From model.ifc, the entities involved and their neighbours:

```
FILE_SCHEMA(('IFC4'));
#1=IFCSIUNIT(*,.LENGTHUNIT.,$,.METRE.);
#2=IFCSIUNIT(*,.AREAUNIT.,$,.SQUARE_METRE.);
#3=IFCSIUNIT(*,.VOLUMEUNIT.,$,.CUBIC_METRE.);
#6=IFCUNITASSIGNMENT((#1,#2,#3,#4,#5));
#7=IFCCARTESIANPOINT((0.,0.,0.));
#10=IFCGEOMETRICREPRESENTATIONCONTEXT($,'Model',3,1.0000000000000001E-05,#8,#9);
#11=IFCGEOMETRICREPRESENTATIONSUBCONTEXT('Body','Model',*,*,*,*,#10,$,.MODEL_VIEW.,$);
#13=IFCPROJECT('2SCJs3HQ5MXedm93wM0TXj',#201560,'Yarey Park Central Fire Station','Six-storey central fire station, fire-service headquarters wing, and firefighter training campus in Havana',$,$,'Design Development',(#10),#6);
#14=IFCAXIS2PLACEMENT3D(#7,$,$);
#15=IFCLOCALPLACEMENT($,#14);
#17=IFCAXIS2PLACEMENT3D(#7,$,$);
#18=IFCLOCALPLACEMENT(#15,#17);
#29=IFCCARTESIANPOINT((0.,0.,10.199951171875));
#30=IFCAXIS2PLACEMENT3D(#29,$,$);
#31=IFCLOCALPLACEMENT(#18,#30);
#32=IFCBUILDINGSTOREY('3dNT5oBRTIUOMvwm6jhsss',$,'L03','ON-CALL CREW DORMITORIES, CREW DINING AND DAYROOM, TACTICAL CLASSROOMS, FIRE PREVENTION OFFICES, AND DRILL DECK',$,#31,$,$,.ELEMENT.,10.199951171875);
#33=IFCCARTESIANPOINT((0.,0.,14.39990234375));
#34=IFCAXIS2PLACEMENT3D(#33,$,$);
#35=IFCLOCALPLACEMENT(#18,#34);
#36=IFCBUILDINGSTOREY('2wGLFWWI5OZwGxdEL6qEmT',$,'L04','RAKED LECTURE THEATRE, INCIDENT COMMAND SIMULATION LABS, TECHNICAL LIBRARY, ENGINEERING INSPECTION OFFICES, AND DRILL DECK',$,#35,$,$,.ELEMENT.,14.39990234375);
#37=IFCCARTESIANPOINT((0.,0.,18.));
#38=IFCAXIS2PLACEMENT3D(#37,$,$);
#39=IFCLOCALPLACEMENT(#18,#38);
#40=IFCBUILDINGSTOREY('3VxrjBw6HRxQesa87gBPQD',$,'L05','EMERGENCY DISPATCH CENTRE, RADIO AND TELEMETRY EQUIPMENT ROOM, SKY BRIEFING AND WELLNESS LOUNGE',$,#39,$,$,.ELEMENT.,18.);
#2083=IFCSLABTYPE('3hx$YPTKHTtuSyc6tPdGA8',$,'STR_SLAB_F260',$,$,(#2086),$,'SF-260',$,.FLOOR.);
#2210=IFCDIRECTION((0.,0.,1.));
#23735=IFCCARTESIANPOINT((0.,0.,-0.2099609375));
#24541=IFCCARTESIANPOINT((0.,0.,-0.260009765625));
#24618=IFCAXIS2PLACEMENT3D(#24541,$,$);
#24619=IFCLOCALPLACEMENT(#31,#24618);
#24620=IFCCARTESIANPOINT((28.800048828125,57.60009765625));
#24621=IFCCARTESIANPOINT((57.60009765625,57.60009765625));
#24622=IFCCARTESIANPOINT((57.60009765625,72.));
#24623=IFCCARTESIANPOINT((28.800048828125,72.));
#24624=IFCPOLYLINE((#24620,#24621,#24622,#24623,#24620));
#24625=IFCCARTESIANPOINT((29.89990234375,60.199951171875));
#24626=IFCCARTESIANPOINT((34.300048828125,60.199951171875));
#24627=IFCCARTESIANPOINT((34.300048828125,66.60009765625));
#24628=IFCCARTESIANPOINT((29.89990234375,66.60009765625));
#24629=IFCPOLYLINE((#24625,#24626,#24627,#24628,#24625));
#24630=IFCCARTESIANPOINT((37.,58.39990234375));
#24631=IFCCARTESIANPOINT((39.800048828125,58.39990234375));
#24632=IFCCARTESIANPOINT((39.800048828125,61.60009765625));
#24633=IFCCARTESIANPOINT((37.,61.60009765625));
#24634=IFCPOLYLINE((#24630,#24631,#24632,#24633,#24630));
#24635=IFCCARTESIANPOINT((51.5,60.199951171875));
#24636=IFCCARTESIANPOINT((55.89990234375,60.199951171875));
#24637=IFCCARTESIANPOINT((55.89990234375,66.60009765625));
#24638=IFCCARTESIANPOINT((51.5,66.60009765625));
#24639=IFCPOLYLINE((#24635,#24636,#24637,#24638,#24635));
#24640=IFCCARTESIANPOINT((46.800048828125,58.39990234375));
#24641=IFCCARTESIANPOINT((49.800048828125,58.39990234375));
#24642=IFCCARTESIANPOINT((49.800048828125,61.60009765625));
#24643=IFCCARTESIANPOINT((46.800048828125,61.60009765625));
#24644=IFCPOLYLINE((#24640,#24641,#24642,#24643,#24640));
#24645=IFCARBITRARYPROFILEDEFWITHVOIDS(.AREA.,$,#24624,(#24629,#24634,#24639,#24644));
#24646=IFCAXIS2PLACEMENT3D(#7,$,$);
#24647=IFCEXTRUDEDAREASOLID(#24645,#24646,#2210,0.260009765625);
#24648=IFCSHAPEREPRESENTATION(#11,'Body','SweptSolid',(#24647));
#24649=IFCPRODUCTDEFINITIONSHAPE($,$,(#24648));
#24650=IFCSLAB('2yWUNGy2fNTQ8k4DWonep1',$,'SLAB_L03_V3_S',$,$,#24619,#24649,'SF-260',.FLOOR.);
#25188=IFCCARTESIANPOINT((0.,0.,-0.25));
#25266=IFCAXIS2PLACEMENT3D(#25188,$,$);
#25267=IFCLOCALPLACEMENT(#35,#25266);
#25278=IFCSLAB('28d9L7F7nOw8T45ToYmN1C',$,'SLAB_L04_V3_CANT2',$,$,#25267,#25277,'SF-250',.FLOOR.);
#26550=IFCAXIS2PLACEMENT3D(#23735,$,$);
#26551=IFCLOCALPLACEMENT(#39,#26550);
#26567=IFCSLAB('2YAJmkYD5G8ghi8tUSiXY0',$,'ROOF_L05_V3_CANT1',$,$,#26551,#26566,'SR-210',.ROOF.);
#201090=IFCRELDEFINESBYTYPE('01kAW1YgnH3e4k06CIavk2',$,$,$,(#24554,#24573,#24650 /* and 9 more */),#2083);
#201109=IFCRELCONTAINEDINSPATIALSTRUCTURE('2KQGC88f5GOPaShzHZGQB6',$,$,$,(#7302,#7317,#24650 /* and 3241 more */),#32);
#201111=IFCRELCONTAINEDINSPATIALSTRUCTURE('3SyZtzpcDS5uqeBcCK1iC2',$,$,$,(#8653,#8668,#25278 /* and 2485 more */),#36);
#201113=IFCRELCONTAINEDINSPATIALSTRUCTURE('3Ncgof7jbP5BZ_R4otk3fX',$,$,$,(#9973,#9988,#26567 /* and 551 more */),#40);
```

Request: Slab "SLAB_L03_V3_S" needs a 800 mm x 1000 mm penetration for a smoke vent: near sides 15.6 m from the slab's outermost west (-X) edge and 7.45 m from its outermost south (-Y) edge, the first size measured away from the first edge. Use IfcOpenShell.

```python
import numpy as np
import ifcopenshell
import ifcopenshell.api.feature
import ifcopenshell.api.geometry
import ifcopenshell.api.root
import ifcopenshell.geom
import ifcopenshell.util.placement
import ifcopenshell.util.representation
import ifcopenshell.util.shape
import ifcopenshell.util.unit

model = ifcopenshell.open("model.ifc")
unit_scale = ifcopenshell.util.unit.calculate_unit_scale(model)
settings = ifcopenshell.geom.settings()


def volume(element):
    """Net volume in cubic metres, openings subtracted."""
    shape = ifcopenshell.geom.create_shape(settings, element)
    return ifcopenshell.util.shape.get_volume(shape.geometry)


slab = model.by_id(24650)
before = volume(slab)

# Extent in the slab's own axes, in metres. The edges named are its -X and -Y sides.
slab_shape = ifcopenshell.geom.create_shape(settings, slab)
vertices = ifcopenshell.util.shape.get_vertices(slab_shape.geometry)
x_min, y_min, bottom = vertices.min(axis=0)
top = vertices[:, 2].max()

opening = ifcopenshell.api.root.create_entity(model, ifc_class="IfcOpeningElement", name="Smoke vent opening", predefined_type="OPENING")
context = ifcopenshell.util.representation.get_context(model, "Model", "Body", "MODEL_VIEW")
width, depth = 0.8, 1
outline = [(0.0, 0.0), (width, 0.0), (width, depth), (0.0, depth), (0.0, 0.0)]
# Overshoot both faces by 50 mm so the cut is clean.
shape = ifcopenshell.api.geometry.add_slab_representation(
    model, context=context, depth=top - bottom + 0.1, polyline=outline
)
ifcopenshell.api.geometry.assign_representation(model, product=opening, representation=shape)

matrix = ifcopenshell.util.placement.get_local_placement(slab.ObjectPlacement)
matrix[:, 3] = matrix @ np.append(np.array([x_min + 15.6, y_min + 7.45, bottom - 0.05]) / unit_scale, 1.0)
ifcopenshell.api.geometry.edit_object_placement(model, product=opening, matrix=matrix, is_si=False)
ifcopenshell.api.feature.add_feature(model, feature=opening, element=slab)

after = volume(slab)

print(f"slab volume {before:.3f} -> {after:.3f} m3")

model.write("model-out.ifc")
```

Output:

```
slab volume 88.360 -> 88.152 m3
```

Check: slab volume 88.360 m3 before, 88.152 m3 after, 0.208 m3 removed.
